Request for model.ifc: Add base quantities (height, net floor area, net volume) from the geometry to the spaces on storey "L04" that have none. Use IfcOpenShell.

First a look at what the model holds.

```python
import ifcopenshell
import ifcopenshell.util.element
import ifcopenshell.util.unit

model = ifcopenshell.open("model.ifc")
print(model.schema)
for unit_type in ("LENGTHUNIT", "AREAUNIT", "VOLUMEUNIT"):
    print(unit_type, ifcopenshell.util.unit.calculate_unit_scale(model, unit_type))
storey = next(s for s in model.by_type("IfcBuildingStorey") if s.Name == "L04")
spaces = [e for e in ifcopenshell.util.element.get_decomposition(storey) if e.is_a("IfcSpace")]
for e in sorted(spaces, key=lambda e: e.id()):
    print(e.id(), e.is_a(), e.Name, list(ifcopenshell.util.element.get_psets(e, qtos_only=True)), sep=" | ")
```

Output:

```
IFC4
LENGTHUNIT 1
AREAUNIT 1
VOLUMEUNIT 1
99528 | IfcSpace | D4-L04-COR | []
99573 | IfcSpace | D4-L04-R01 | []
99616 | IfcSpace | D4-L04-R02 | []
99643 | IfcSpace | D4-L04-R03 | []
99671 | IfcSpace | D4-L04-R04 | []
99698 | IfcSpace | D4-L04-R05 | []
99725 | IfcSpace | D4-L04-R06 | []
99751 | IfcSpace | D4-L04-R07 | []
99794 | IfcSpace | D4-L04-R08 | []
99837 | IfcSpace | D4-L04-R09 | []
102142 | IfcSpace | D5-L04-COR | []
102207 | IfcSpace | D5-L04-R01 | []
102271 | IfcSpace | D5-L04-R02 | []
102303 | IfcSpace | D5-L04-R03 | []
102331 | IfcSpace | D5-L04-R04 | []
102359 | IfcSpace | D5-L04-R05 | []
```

```python
import ifcopenshell
import ifcopenshell.api.pset
import ifcopenshell.geom
import ifcopenshell.util.element
import ifcopenshell.util.shape
import ifcopenshell.util.unit

model = ifcopenshell.open("model.ifc")
unit_scale = ifcopenshell.util.unit.calculate_unit_scale(model)
area_scale = ifcopenshell.util.unit.calculate_unit_scale(model, "AREAUNIT")
volume_scale = ifcopenshell.util.unit.calculate_unit_scale(model, "VOLUMEUNIT")
settings = ifcopenshell.geom.settings()

storey = next(s for s in model.by_type("IfcBuildingStorey") if s.Name == "L04")
spaces = [e for e in ifcopenshell.util.element.get_decomposition(storey) if e.is_a("IfcSpace")]

for e in sorted(spaces, key=lambda e: e.id()):
    if ifcopenshell.util.element.get_psets(e, qtos_only=True, should_inherit=False):
        continue
    # Geometry comes back in metres, in the element's own axes.
    shape = ifcopenshell.geom.create_shape(settings, e)
    values = {
        "Height": ifcopenshell.util.shape.get_z(shape.geometry) / unit_scale,
        "NetFloorArea": ifcopenshell.util.shape.get_footprint_area(shape.geometry) / area_scale,
        "NetVolume": ifcopenshell.util.shape.get_volume(shape.geometry) / volume_scale,
    }
    qto = ifcopenshell.api.pset.add_qto(model, product=e, name="Qto_SpaceBaseQuantities")
    ifcopenshell.api.pset.edit_qto(model, qto=qto, properties=values)
    print(e.id(), {k: round(v, 3) for k, v in values.items()})

model.write("model-out.ifc")
```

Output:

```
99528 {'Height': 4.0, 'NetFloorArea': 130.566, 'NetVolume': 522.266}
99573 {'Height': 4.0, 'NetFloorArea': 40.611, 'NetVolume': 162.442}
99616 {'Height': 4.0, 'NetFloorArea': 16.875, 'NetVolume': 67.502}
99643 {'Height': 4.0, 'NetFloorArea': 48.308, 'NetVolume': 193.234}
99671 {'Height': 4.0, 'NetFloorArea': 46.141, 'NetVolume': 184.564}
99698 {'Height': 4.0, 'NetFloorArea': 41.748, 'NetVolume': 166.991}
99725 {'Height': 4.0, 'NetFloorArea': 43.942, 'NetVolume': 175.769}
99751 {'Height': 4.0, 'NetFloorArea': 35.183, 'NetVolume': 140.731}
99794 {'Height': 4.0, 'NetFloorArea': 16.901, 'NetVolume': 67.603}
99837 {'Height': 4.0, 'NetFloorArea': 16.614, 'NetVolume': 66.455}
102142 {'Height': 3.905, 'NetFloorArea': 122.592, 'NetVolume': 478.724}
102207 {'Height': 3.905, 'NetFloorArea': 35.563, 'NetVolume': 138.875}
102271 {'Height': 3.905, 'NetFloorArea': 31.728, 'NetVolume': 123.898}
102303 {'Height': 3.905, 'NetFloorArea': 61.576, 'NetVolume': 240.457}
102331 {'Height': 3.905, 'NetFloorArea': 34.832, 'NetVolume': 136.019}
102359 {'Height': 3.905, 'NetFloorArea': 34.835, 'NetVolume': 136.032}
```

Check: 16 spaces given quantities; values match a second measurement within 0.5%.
